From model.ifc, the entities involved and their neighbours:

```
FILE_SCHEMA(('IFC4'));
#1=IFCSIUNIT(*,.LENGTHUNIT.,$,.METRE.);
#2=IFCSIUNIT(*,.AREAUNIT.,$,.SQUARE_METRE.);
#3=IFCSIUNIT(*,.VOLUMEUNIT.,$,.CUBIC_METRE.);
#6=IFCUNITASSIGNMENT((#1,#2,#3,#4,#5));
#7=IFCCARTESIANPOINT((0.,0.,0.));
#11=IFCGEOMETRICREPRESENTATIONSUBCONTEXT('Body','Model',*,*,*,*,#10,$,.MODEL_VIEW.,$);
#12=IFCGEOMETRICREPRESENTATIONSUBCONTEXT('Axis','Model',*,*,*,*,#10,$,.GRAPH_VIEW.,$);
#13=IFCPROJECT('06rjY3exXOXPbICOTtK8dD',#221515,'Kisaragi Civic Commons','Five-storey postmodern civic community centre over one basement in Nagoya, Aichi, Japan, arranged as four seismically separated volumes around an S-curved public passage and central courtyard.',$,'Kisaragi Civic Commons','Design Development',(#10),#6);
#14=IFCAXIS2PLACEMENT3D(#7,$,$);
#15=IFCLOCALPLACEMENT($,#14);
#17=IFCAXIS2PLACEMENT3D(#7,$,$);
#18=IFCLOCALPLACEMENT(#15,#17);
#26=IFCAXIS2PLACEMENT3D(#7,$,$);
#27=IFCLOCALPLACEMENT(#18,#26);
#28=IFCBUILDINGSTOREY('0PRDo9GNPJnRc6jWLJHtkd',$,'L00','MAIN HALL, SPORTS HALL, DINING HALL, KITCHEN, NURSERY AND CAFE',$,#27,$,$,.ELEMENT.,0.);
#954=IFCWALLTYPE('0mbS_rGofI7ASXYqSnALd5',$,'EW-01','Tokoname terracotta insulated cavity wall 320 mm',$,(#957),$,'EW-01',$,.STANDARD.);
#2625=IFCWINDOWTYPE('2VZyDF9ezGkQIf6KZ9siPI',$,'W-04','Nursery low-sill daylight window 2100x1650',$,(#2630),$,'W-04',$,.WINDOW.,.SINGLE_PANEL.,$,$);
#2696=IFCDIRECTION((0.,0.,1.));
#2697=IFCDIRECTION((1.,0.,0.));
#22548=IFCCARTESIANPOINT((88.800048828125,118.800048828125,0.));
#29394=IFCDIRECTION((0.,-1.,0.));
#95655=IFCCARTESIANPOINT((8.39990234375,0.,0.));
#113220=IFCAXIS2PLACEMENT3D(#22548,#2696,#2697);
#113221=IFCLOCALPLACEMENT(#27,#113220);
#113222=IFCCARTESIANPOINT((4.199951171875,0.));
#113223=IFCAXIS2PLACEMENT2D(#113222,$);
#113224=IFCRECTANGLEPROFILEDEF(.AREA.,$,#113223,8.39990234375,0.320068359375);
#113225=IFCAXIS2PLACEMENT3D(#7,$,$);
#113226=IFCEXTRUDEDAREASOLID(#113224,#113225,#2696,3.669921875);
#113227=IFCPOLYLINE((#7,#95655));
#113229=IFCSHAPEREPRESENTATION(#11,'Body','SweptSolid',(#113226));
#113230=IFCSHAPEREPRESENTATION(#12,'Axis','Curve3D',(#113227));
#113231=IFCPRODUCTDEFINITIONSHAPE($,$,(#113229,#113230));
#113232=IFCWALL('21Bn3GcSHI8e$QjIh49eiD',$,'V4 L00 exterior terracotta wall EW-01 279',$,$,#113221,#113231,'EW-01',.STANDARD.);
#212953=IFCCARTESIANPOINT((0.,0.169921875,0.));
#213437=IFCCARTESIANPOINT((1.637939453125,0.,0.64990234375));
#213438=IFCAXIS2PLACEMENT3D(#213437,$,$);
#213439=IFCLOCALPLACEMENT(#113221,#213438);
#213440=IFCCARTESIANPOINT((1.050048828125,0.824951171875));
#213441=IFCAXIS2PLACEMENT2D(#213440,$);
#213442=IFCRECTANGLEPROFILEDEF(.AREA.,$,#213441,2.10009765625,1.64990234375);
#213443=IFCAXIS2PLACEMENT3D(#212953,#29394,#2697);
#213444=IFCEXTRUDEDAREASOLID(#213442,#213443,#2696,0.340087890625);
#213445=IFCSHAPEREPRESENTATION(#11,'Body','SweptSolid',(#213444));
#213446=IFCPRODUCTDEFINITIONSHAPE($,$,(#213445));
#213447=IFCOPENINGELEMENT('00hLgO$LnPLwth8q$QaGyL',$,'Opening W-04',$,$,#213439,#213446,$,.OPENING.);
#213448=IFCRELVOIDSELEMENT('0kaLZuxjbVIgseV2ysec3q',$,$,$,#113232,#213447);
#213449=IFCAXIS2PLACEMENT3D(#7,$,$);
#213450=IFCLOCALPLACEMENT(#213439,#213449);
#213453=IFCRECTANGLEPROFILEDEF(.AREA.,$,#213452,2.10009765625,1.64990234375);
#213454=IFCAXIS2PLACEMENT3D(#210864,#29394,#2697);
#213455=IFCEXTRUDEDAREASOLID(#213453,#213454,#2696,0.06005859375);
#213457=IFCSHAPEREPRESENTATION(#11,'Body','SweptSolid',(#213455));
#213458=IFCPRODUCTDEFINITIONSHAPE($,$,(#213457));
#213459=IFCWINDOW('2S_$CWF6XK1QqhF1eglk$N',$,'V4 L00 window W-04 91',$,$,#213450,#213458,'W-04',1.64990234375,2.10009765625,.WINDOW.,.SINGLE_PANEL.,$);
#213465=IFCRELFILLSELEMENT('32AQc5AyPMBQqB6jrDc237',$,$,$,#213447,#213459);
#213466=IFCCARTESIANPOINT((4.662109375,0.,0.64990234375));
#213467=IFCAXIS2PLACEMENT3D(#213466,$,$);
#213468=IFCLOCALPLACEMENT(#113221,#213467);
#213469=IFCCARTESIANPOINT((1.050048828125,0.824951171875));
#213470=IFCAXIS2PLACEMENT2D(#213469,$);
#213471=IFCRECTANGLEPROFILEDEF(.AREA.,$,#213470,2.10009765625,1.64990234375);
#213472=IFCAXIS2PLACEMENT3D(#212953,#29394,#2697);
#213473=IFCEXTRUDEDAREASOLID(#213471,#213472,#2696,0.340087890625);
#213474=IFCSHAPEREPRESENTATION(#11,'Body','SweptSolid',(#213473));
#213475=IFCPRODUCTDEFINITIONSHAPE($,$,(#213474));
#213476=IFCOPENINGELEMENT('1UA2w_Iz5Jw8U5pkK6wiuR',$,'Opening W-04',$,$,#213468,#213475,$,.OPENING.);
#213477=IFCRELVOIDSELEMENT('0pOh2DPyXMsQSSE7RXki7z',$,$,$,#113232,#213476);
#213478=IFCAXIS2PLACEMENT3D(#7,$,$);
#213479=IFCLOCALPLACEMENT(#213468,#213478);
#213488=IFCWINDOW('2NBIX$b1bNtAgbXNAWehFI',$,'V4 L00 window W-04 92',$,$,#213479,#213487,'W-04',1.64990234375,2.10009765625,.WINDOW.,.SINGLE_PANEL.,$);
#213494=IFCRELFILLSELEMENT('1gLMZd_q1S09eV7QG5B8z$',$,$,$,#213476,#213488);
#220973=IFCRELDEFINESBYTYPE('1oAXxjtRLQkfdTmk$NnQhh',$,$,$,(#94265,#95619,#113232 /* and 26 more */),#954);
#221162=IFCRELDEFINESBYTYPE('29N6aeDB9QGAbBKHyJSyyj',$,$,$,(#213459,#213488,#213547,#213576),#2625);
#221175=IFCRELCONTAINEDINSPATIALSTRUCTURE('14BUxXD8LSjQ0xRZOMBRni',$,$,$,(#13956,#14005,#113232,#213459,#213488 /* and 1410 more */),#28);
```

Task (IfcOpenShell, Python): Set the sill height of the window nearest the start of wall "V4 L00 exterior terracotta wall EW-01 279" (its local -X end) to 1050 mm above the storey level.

```python
import numpy as np
import ifcopenshell
import ifcopenshell.api.geometry
import ifcopenshell.geom
import ifcopenshell.util.element
import ifcopenshell.util.placement
import ifcopenshell.util.shape
import ifcopenshell.util.unit

model = ifcopenshell.open("model.ifc")
unit_scale = ifcopenshell.util.unit.calculate_unit_scale(model)

window = model.by_guid("2S_$CWF6XK1QqhF1eglk$N")
opening = window.FillsVoids[0].RelatingOpeningElement
storey = ifcopenshell.util.element.get_container(window, ifc_class="IfcBuildingStorey")
level = ifcopenshell.util.placement.get_local_placement(storey.ObjectPlacement)[2, 3]

# The opening's origin need not be at the sill, so measure its lowest point.
shape = ifcopenshell.geom.create_shape(ifcopenshell.geom.settings(), opening)
bottom = ifcopenshell.util.shape.get_shape_bottom_elevation(shape, shape.geometry) / unit_scale
dz = level + 1.05 / unit_scale - bottom

shift = np.array([0.0, 0.0, dz])
# The window is placed relative to its opening, so it follows when the opening moves.
matrix = ifcopenshell.util.placement.get_local_placement(opening.ObjectPlacement)
matrix[:3, 3] += shift
ifcopenshell.api.geometry.edit_object_placement(
    model, product=opening, matrix=matrix, is_si=False, should_transform_children=True
)

print(f"moved by {dz * unit_scale:+.3f} m")

model.write("model_edited.ifc")
```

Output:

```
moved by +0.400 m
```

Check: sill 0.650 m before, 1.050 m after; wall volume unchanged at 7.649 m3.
